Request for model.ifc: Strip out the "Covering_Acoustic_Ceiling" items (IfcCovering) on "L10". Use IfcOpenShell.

First a look at what the model holds.

```python
import ifcopenshell
import ifcopenshell.util.element

model = ifcopenshell.open("model.ifc")
print(model.schema)
storey = next(s for s in model.by_type("IfcBuildingStorey") if s.Name == "L10")
coverings = [e for e in ifcopenshell.util.element.get_decomposition(storey) if e.is_a("IfcCovering")]
seen = {}
for e in coverings:
    element_type = ifcopenshell.util.element.get_type(e)
    name = element_type.Name if element_type not in (None, e) else None
    seen[name] = seen.get(name, 0) + 1
for name, count in sorted(seen.items(), key=str):
    print(count, "x", name)
```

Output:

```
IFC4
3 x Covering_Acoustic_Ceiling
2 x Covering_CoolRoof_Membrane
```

```python
import ifcopenshell
import ifcopenshell.api.root
import ifcopenshell.util.element

model = ifcopenshell.open("model.ifc")

storey = next(s for s in model.by_type("IfcBuildingStorey") if s.Name == "L10")
coverings = [e for e in ifcopenshell.util.element.get_decomposition(storey) if e.is_a("IfcCovering")]
targets = [e for e in coverings if (t := ifcopenshell.util.element.get_type(e)) not in (None, e) and t.Name == "Covering_Acoustic_Ceiling"]

for e in targets:
    ifcopenshell.api.root.remove_product(model, product=e)
print(len(targets), "removed")

model.write("model-out.ifc")
```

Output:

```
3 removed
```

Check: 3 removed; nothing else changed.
